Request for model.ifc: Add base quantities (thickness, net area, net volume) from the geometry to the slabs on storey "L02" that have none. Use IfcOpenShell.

First a look at what the model holds.

```python
import ifcopenshell
import ifcopenshell.util.element
import ifcopenshell.util.unit

model = ifcopenshell.open("model.ifc")
print(model.schema)
for unit_type in ("LENGTHUNIT", "AREAUNIT", "VOLUMEUNIT"):
    print(unit_type, ifcopenshell.util.unit.calculate_unit_scale(model, unit_type))
storey = next(s for s in model.by_type("IfcBuildingStorey") if s.Name == "L02")
slabs = [e for e in ifcopenshell.util.element.get_decomposition(storey) if e.is_a("IfcSlab")]
for e in sorted(slabs, key=lambda e: e.id()):
    print(e.id(), e.is_a(), e.Name, list(ifcopenshell.util.element.get_psets(e, qtos_only=True)), sep=" | ")
```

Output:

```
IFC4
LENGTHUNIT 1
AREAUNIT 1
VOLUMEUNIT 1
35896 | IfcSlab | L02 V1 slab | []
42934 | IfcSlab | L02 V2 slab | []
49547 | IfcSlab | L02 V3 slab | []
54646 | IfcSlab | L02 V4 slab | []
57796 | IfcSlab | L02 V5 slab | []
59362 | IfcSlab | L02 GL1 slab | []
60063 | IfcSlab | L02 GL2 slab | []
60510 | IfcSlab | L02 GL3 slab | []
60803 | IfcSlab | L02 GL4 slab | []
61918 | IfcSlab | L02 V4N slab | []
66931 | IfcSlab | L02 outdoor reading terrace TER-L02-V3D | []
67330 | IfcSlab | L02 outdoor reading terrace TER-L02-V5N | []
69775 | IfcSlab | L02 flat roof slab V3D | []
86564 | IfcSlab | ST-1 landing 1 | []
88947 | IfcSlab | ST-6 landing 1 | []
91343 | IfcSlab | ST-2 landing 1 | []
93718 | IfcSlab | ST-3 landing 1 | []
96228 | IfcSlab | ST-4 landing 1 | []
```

```python
import ifcopenshell
import ifcopenshell.api.pset
import ifcopenshell.geom
import ifcopenshell.util.element
import ifcopenshell.util.shape
import ifcopenshell.util.unit

model = ifcopenshell.open("model.ifc")
unit_scale = ifcopenshell.util.unit.calculate_unit_scale(model)
area_scale = ifcopenshell.util.unit.calculate_unit_scale(model, "AREAUNIT")
volume_scale = ifcopenshell.util.unit.calculate_unit_scale(model, "VOLUMEUNIT")
settings = ifcopenshell.geom.settings()

storey = next(s for s in model.by_type("IfcBuildingStorey") if s.Name == "L02")
slabs = [e for e in ifcopenshell.util.element.get_decomposition(storey) if e.is_a("IfcSlab")]

for e in sorted(slabs, key=lambda e: e.id()):
    if ifcopenshell.util.element.get_psets(e, qtos_only=True, should_inherit=False):
        continue
    # Geometry comes back in metres, in the element's own axes.
    shape = ifcopenshell.geom.create_shape(settings, e)
    values = {
        "Width": ifcopenshell.util.shape.get_z(shape.geometry) / unit_scale,
        "NetArea": ifcopenshell.util.shape.get_footprint_area(shape.geometry) / area_scale,
        "NetVolume": ifcopenshell.util.shape.get_volume(shape.geometry) / volume_scale,
    }
    qto = ifcopenshell.api.pset.add_qto(model, product=e, name="Qto_SlabBaseQuantities")
    ifcopenshell.api.pset.edit_qto(model, qto=qto, properties=values)
    print(e.id(), {k: round(v, 3) for k, v in values.items()})

model.write("model_edited.ifc")
```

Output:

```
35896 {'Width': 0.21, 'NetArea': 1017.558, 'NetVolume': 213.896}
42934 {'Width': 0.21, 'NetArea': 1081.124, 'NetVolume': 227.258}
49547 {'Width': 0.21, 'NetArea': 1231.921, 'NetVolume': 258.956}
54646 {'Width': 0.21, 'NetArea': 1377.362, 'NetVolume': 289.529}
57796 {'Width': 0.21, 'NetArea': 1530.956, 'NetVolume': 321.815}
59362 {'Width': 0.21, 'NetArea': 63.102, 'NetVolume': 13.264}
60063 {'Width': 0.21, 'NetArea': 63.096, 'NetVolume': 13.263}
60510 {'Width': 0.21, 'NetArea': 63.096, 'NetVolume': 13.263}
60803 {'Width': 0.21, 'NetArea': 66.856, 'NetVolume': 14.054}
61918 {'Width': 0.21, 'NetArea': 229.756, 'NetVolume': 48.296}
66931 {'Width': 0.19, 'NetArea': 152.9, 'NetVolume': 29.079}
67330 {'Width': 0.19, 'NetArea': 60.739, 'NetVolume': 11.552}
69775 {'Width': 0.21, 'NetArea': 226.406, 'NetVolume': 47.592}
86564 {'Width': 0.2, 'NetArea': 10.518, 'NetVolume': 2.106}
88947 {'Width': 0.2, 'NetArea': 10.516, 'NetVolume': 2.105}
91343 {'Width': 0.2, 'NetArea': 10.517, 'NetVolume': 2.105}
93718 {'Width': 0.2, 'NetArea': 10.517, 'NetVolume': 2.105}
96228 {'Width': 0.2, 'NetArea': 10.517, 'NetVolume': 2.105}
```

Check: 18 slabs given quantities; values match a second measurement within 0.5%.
